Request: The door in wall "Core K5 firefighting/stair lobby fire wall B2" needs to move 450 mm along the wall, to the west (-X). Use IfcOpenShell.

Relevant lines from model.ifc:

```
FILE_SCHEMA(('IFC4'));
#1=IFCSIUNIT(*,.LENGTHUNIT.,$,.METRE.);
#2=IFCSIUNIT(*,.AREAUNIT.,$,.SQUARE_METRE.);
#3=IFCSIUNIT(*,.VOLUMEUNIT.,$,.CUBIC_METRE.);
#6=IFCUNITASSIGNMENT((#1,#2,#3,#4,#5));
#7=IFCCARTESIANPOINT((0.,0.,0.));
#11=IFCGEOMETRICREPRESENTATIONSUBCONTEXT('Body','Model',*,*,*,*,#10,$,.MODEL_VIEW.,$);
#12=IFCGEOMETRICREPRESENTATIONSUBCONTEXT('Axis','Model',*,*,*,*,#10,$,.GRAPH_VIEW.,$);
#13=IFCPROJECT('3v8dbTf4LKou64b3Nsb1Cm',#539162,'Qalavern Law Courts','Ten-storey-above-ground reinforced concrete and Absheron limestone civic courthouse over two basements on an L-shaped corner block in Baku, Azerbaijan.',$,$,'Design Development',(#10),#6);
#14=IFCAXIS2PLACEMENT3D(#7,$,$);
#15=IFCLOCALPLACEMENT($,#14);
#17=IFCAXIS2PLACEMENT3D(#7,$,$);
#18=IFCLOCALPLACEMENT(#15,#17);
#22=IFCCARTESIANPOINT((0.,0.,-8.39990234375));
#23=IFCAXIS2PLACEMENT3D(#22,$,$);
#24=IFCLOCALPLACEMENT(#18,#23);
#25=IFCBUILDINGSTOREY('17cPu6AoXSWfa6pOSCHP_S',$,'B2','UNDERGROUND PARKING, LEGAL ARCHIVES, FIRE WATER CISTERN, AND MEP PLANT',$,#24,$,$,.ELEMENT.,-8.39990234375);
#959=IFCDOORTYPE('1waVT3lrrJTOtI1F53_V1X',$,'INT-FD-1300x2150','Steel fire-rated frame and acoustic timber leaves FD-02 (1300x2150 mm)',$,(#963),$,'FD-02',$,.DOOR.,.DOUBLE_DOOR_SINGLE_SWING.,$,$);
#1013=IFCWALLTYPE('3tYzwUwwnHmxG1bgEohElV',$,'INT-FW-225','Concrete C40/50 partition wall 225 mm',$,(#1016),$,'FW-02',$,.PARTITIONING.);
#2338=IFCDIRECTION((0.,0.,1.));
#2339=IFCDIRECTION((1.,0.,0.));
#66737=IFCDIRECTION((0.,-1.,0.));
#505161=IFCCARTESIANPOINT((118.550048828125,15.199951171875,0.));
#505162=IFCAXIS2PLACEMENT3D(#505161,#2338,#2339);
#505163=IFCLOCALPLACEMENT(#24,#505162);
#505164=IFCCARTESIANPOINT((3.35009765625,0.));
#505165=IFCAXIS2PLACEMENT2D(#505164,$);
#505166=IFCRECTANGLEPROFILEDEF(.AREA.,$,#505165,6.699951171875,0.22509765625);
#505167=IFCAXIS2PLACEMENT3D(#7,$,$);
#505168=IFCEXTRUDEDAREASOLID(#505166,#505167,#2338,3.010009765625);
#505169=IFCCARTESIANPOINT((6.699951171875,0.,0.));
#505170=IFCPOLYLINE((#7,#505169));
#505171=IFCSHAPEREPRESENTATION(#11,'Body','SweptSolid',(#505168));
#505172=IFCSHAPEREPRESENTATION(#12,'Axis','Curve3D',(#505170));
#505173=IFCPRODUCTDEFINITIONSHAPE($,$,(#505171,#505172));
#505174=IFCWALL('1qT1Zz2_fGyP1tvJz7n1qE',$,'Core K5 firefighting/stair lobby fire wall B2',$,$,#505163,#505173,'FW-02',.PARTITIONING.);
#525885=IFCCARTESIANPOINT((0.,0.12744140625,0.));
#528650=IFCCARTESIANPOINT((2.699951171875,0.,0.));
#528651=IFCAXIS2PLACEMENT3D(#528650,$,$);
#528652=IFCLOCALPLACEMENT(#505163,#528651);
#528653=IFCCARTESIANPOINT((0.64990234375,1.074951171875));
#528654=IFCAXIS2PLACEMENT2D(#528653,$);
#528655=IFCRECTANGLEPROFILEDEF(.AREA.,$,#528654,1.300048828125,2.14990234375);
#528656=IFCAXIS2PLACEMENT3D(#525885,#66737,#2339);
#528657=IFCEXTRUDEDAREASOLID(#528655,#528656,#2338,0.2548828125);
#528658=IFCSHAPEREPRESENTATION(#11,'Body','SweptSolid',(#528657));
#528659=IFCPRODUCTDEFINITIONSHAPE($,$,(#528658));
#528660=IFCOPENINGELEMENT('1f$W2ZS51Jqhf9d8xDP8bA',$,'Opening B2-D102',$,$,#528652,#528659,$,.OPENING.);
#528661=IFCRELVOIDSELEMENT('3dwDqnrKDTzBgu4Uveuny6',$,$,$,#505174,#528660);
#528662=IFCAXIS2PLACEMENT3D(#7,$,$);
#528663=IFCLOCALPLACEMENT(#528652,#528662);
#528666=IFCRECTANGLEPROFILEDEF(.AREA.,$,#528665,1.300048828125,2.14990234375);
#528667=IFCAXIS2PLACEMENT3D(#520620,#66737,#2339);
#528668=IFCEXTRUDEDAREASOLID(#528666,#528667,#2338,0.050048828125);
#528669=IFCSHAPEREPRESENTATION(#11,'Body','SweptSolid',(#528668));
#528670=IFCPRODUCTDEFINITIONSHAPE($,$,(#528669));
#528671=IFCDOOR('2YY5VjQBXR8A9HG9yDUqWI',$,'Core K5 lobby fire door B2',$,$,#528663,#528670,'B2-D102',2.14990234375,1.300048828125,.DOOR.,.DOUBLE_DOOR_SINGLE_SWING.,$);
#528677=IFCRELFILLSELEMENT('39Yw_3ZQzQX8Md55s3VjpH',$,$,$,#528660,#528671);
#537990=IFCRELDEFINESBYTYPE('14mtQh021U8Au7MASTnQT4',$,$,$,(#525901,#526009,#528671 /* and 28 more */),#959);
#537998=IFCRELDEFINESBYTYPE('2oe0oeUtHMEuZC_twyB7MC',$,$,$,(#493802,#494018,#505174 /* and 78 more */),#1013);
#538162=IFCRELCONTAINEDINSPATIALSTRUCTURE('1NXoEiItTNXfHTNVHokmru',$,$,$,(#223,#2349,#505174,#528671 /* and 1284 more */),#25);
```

```python
import ifcopenshell
import ifcopenshell.api.geometry
import ifcopenshell.util.placement

model = ifcopenshell.open("model.ifc")

door = model.by_guid("2YY5VjQBXR8A9HG9yDUqWI")
opening = door.FillsVoids[0].RelatingOpeningElement
wall = opening.VoidsElements[0].RelatingBuildingElement

wall_matrix = ifcopenshell.util.placement.get_local_placement(wall.ObjectPlacement)
shift = wall_matrix[:3, 0] * -0.45
before = ifcopenshell.util.placement.get_local_placement(door.ObjectPlacement)[:3, 3].copy()

# The door is placed relative to its opening, so it follows when the opening moves.
matrix = ifcopenshell.util.placement.get_local_placement(opening.ObjectPlacement)
matrix[:3, 3] += shift
ifcopenshell.api.geometry.edit_object_placement(
    model, product=opening, matrix=matrix, is_si=False, should_transform_children=True
)

after = ifcopenshell.util.placement.get_local_placement(door.ObjectPlacement)[:3, 3]
print("door moved by", (after - before).round(3) + 0.0)

model.write("model_updated.ifc")
```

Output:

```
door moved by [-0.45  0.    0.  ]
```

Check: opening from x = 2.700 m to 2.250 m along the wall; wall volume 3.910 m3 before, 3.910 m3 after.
